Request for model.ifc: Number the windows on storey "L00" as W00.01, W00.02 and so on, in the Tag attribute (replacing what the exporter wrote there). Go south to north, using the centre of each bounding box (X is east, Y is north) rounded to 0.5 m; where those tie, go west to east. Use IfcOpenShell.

First a look at what the model holds.

```python
import ifcopenshell
import ifcopenshell.util.element
import ifcopenshell.util.placement

model = ifcopenshell.open("model.ifc")
print(model.schema)
storey = next(s for s in model.by_type("IfcBuildingStorey") if s.Name == "L00")
windows = [e for e in ifcopenshell.util.element.get_decomposition(storey) if e.is_a("IfcWindow")]
for e in sorted(windows, key=lambda e: e.id()):
    origin = ifcopenshell.util.placement.get_local_placement(e.ObjectPlacement)[:3, 3]
    print(e.id(), e.Tag, e.Name, origin.round(2) + 0.0, sep=" | ")
```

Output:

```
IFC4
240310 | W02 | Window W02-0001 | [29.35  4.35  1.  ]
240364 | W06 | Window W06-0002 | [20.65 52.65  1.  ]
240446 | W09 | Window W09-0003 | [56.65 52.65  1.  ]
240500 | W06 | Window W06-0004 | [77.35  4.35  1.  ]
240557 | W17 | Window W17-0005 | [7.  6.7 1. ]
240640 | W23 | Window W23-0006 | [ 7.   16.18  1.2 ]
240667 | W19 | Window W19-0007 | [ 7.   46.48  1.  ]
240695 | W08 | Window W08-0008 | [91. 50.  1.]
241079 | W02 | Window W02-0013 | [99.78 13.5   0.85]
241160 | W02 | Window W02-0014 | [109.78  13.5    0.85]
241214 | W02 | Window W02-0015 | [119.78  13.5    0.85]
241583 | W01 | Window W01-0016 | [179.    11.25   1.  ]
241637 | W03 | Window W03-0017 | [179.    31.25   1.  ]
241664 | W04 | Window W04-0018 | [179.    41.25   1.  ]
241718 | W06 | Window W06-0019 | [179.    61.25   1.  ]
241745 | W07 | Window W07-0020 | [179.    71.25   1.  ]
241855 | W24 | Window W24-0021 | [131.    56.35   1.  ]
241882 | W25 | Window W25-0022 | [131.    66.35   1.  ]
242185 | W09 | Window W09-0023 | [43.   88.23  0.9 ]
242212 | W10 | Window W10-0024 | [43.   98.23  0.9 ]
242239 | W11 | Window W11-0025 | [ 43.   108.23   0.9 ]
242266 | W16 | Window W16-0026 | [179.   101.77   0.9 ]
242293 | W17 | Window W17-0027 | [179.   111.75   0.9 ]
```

```python
import ifcopenshell
import ifcopenshell.geom
import ifcopenshell.util.element
import ifcopenshell.util.shape

model = ifcopenshell.open("model.ifc")
settings = ifcopenshell.geom.settings()
settings.set("use-world-coords", True)


def centre(element):
    shape = ifcopenshell.geom.create_shape(settings, element)
    return ifcopenshell.util.shape.get_bbox_centroid(shape.geometry)


storey = next(s for s in model.by_type("IfcBuildingStorey") if s.Name == "L00")
windows = [e for e in ifcopenshell.util.element.get_decomposition(storey) if e.is_a("IfcWindow")]

# Insertion points can sit at a corner or the storey origin, so sort by the geometry (in metres).
centres = {e: centre(e) for e in windows}
windows.sort(key=lambda e: (round(centres[e][1] / 0.5), centres[e][0]))

for i, e in enumerate(windows, start=1):
    number = f"W00.{i:02d}"
    e.Tag = number
    print(e.id(), number)

model.write("model_rev.ifc")
```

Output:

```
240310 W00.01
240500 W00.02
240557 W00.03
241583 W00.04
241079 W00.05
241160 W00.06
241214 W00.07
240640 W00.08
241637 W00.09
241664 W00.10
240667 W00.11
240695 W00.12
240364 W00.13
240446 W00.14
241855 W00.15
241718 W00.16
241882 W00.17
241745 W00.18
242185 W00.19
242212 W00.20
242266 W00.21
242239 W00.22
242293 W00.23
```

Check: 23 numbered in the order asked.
